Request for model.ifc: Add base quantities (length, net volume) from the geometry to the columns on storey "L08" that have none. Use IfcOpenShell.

First a look at what the model holds.

```python
import ifcopenshell
import ifcopenshell.util.element
import ifcopenshell.util.unit

model = ifcopenshell.open("model.ifc")
print(model.schema)
for unit_type in ("LENGTHUNIT", "AREAUNIT", "VOLUMEUNIT"):
    print(unit_type, ifcopenshell.util.unit.calculate_unit_scale(model, unit_type))
storey = next(s for s in model.by_type("IfcBuildingStorey") if s.Name == "L08")
columns = [e for e in ifcopenshell.util.element.get_decomposition(storey) if e.is_a("IfcColumn")]
for e in sorted(columns, key=lambda e: e.id()):
    print(e.id(), e.is_a(), e.Name, list(ifcopenshell.util.element.get_psets(e, qtos_only=True)), sep=" | ")
```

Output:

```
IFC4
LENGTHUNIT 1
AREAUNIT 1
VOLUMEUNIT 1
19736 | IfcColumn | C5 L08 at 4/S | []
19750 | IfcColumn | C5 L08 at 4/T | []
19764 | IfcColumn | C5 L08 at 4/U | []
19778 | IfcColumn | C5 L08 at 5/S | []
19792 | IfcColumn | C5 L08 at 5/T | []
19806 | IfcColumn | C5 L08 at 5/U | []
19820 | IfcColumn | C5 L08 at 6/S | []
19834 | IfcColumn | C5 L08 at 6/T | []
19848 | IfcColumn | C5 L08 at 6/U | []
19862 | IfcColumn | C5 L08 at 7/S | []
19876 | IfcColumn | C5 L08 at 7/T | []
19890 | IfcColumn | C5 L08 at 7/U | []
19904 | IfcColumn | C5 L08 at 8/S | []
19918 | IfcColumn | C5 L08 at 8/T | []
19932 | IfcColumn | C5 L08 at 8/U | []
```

```python
import ifcopenshell
import ifcopenshell.api.pset
import ifcopenshell.geom
import ifcopenshell.util.element
import ifcopenshell.util.shape
import ifcopenshell.util.unit

model = ifcopenshell.open("model.ifc")
unit_scale = ifcopenshell.util.unit.calculate_unit_scale(model)
volume_scale = ifcopenshell.util.unit.calculate_unit_scale(model, "VOLUMEUNIT")
settings = ifcopenshell.geom.settings()

storey = next(s for s in model.by_type("IfcBuildingStorey") if s.Name == "L08")
columns = [e for e in ifcopenshell.util.element.get_decomposition(storey) if e.is_a("IfcColumn")]

for e in sorted(columns, key=lambda e: e.id()):
    if ifcopenshell.util.element.get_psets(e, qtos_only=True, should_inherit=False):
        continue
    # Geometry comes back in metres, in the element's own axes.
    shape = ifcopenshell.geom.create_shape(settings, e)
    values = {
        "Length": ifcopenshell.util.shape.get_z(shape.geometry) / unit_scale,
        "NetVolume": ifcopenshell.util.shape.get_volume(shape.geometry) / volume_scale,
    }
    qto = ifcopenshell.api.pset.add_qto(model, product=e, name="Qto_ColumnBaseQuantities")
    ifcopenshell.api.pset.edit_qto(model, qto=qto, properties=values)
    print(e.id(), {k: round(v, 3) for k, v in values.items()})

model.write("model_rev.ifc")
```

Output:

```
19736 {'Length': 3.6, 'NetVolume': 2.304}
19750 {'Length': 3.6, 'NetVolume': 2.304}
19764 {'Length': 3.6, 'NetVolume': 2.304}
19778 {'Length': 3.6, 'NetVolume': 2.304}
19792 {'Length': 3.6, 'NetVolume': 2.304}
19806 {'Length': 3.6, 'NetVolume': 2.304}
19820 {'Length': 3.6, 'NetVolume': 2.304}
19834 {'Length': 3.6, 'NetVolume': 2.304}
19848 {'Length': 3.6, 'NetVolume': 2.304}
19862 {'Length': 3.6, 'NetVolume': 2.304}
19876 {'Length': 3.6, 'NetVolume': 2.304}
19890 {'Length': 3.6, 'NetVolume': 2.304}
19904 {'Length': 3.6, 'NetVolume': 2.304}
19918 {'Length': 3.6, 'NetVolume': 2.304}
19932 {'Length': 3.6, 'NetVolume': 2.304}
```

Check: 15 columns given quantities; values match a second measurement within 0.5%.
